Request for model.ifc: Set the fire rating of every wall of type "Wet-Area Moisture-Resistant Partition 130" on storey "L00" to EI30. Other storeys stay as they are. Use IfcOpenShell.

First a look at what the model holds.

```python
import ifcopenshell
import ifcopenshell.util.element

model = ifcopenshell.open("model.ifc")
print(model.schema)
storey = next(s for s in model.by_type("IfcBuildingStorey") if s.Name == "L00")
walls = [e for e in ifcopenshell.util.element.get_decomposition(storey) if e.is_a("IfcWall")]
seen = {}
for e in walls:
    element_type = ifcopenshell.util.element.get_type(e)
    key = (element_type.Name if element_type != e and element_type else None, ifcopenshell.util.element.get_pset(e, "Pset_WallCommon", "FireRating"))
    seen[key] = seen.get(key, 0) + 1
for (name, value), count in sorted(seen.items(), key=str):
    print(count, "x", name, "|", value)
```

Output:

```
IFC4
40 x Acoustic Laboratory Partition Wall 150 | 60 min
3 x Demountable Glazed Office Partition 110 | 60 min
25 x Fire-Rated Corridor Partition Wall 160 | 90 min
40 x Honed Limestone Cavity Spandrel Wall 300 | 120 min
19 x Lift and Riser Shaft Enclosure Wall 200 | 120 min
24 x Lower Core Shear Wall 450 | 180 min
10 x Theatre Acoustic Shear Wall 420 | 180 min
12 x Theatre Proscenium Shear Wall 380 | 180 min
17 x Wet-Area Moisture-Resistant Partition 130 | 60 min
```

```python
import ifcopenshell
import ifcopenshell.api.pset
import ifcopenshell.util.element

model = ifcopenshell.open("model.ifc")

storey = next(s for s in model.by_type("IfcBuildingStorey") if s.Name == "L00")
walls = [e for e in ifcopenshell.util.element.get_decomposition(storey) if e.is_a("IfcWall")]

count = 0
for e in walls:
    element_type = ifcopenshell.util.element.get_type(e)
    if element_type in (None, e) or element_type.Name != "Wet-Area Moisture-Resistant Partition 130":
        continue
    # add_pset returns the element's existing set when there is one.
    pset = ifcopenshell.api.pset.add_pset(model, product=e, name="Pset_WallCommon")
    ifcopenshell.api.pset.edit_pset(model, pset=pset, properties={"FireRating": "EI30"})
    count += 1

print(count, "walls updated")

model.write("model-out.ifc")
```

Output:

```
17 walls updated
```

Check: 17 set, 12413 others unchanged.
